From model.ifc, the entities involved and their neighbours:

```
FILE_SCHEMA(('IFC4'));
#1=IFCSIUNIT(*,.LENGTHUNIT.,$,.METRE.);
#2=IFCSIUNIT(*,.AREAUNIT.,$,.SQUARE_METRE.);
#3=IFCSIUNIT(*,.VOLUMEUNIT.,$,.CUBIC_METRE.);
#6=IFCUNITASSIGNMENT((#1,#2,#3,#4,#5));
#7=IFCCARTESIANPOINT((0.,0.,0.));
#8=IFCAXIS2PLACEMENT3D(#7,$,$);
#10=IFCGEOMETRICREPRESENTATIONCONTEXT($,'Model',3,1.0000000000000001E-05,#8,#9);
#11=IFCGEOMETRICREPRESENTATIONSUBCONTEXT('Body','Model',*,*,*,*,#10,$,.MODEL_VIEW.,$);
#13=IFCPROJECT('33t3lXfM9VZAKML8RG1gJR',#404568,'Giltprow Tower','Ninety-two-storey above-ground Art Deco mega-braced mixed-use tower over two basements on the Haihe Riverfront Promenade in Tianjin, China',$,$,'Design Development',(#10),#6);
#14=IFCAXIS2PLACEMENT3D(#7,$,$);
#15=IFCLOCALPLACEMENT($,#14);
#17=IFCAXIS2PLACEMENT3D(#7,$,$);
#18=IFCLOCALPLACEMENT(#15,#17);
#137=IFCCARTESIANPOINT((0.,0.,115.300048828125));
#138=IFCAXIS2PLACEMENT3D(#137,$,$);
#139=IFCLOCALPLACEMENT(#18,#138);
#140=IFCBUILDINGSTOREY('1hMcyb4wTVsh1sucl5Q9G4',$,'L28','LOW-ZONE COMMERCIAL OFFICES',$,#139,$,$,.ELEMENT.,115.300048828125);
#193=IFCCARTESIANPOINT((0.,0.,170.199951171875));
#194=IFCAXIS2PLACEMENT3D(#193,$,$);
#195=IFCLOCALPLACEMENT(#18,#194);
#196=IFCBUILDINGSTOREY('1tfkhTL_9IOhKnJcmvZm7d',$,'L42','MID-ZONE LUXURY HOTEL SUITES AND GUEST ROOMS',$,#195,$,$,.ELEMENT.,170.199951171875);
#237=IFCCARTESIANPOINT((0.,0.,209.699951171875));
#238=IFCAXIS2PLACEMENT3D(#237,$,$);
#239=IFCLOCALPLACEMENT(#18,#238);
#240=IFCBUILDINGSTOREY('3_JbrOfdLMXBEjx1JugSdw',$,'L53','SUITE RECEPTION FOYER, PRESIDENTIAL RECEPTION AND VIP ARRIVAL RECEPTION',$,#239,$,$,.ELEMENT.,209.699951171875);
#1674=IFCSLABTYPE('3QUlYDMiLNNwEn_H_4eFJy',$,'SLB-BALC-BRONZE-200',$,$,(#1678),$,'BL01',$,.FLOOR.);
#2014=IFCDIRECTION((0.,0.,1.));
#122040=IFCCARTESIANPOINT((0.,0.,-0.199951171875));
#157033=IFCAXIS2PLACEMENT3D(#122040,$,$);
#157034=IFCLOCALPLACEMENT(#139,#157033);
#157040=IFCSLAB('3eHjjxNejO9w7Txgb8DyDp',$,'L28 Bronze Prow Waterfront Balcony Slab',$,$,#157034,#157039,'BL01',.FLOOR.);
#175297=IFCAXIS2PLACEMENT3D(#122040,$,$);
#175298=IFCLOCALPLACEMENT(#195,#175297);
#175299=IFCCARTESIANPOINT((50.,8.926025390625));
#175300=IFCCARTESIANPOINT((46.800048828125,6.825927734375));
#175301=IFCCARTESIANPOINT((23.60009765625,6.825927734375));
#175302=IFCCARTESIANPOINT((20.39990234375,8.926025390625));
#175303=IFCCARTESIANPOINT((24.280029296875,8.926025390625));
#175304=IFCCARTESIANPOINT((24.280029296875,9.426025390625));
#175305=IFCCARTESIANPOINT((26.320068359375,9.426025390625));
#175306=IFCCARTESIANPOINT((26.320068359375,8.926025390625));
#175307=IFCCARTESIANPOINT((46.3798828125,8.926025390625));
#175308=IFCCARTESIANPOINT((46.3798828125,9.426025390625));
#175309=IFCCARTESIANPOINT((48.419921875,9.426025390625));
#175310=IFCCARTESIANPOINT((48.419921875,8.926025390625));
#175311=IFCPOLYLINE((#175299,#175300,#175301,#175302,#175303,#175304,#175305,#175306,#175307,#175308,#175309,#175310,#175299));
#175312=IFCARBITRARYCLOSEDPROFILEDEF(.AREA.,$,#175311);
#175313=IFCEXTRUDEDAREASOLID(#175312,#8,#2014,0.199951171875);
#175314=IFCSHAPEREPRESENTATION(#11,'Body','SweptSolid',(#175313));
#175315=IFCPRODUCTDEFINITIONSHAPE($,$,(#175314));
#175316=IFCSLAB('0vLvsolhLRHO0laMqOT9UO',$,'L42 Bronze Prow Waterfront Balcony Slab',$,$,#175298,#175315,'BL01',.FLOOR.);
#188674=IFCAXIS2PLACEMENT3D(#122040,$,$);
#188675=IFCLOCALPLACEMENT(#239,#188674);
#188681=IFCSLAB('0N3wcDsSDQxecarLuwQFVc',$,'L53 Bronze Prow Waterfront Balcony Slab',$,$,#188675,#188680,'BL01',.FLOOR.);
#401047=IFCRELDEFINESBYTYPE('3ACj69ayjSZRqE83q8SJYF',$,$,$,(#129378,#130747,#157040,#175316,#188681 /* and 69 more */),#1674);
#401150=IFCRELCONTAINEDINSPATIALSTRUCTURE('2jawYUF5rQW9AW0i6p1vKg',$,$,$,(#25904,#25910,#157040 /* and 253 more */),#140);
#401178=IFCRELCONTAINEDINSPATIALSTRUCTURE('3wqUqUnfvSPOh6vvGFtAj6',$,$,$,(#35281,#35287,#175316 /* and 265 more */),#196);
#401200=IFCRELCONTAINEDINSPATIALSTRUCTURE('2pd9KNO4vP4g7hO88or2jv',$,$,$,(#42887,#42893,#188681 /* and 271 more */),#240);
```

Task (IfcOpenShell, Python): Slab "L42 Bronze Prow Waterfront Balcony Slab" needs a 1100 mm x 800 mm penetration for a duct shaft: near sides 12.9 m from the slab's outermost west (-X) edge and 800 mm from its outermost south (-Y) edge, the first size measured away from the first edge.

```python
import numpy as np
import ifcopenshell
import ifcopenshell.api.feature
import ifcopenshell.api.geometry
import ifcopenshell.api.root
import ifcopenshell.geom
import ifcopenshell.util.placement
import ifcopenshell.util.representation
import ifcopenshell.util.shape
import ifcopenshell.util.unit

model = ifcopenshell.open("model.ifc")
unit_scale = ifcopenshell.util.unit.calculate_unit_scale(model)
settings = ifcopenshell.geom.settings()


def volume(element):
    """Net volume in cubic metres, openings subtracted."""
    shape = ifcopenshell.geom.create_shape(settings, element)
    return ifcopenshell.util.shape.get_volume(shape.geometry)


slab = model.by_guid("0vLvsolhLRHO0laMqOT9UO")
before = volume(slab)

# Extent in the slab's own axes, in metres. The edges named are its -X and -Y sides.
slab_shape = ifcopenshell.geom.create_shape(settings, slab)
vertices = ifcopenshell.util.shape.get_vertices(slab_shape.geometry)
x_min, y_min, bottom = vertices.min(axis=0)
top = vertices[:, 2].max()

opening = ifcopenshell.api.root.create_entity(model, ifc_class="IfcOpeningElement", name="Duct shaft opening", predefined_type="OPENING")
context = ifcopenshell.util.representation.get_context(model, "Model", "Body", "MODEL_VIEW")
width, depth = 1.1, 0.8
outline = [(0.0, 0.0), (width, 0.0), (width, depth), (0.0, depth), (0.0, 0.0)]
# Overshoot both faces by 50 mm so the cut is clean.
shape = ifcopenshell.api.geometry.add_slab_representation(
    model, context=context, depth=top - bottom + 0.1, polyline=outline
)
ifcopenshell.api.geometry.assign_representation(model, product=opening, representation=shape)

matrix = ifcopenshell.util.placement.get_local_placement(slab.ObjectPlacement)
matrix[:, 3] = matrix @ np.append(np.array([x_min + 12.9, y_min + 0.8, bottom - 0.05]) / unit_scale, 1.0)
ifcopenshell.api.geometry.edit_object_placement(model, product=opening, matrix=matrix, is_si=False)
ifcopenshell.api.feature.add_feature(model, feature=opening, element=slab)

after = volume(slab)

print(f"slab volume {before:.3f} -> {after:.3f} m3")

model.write("model_v2.ifc")
```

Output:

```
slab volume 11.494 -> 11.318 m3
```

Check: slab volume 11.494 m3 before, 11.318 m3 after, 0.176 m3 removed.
